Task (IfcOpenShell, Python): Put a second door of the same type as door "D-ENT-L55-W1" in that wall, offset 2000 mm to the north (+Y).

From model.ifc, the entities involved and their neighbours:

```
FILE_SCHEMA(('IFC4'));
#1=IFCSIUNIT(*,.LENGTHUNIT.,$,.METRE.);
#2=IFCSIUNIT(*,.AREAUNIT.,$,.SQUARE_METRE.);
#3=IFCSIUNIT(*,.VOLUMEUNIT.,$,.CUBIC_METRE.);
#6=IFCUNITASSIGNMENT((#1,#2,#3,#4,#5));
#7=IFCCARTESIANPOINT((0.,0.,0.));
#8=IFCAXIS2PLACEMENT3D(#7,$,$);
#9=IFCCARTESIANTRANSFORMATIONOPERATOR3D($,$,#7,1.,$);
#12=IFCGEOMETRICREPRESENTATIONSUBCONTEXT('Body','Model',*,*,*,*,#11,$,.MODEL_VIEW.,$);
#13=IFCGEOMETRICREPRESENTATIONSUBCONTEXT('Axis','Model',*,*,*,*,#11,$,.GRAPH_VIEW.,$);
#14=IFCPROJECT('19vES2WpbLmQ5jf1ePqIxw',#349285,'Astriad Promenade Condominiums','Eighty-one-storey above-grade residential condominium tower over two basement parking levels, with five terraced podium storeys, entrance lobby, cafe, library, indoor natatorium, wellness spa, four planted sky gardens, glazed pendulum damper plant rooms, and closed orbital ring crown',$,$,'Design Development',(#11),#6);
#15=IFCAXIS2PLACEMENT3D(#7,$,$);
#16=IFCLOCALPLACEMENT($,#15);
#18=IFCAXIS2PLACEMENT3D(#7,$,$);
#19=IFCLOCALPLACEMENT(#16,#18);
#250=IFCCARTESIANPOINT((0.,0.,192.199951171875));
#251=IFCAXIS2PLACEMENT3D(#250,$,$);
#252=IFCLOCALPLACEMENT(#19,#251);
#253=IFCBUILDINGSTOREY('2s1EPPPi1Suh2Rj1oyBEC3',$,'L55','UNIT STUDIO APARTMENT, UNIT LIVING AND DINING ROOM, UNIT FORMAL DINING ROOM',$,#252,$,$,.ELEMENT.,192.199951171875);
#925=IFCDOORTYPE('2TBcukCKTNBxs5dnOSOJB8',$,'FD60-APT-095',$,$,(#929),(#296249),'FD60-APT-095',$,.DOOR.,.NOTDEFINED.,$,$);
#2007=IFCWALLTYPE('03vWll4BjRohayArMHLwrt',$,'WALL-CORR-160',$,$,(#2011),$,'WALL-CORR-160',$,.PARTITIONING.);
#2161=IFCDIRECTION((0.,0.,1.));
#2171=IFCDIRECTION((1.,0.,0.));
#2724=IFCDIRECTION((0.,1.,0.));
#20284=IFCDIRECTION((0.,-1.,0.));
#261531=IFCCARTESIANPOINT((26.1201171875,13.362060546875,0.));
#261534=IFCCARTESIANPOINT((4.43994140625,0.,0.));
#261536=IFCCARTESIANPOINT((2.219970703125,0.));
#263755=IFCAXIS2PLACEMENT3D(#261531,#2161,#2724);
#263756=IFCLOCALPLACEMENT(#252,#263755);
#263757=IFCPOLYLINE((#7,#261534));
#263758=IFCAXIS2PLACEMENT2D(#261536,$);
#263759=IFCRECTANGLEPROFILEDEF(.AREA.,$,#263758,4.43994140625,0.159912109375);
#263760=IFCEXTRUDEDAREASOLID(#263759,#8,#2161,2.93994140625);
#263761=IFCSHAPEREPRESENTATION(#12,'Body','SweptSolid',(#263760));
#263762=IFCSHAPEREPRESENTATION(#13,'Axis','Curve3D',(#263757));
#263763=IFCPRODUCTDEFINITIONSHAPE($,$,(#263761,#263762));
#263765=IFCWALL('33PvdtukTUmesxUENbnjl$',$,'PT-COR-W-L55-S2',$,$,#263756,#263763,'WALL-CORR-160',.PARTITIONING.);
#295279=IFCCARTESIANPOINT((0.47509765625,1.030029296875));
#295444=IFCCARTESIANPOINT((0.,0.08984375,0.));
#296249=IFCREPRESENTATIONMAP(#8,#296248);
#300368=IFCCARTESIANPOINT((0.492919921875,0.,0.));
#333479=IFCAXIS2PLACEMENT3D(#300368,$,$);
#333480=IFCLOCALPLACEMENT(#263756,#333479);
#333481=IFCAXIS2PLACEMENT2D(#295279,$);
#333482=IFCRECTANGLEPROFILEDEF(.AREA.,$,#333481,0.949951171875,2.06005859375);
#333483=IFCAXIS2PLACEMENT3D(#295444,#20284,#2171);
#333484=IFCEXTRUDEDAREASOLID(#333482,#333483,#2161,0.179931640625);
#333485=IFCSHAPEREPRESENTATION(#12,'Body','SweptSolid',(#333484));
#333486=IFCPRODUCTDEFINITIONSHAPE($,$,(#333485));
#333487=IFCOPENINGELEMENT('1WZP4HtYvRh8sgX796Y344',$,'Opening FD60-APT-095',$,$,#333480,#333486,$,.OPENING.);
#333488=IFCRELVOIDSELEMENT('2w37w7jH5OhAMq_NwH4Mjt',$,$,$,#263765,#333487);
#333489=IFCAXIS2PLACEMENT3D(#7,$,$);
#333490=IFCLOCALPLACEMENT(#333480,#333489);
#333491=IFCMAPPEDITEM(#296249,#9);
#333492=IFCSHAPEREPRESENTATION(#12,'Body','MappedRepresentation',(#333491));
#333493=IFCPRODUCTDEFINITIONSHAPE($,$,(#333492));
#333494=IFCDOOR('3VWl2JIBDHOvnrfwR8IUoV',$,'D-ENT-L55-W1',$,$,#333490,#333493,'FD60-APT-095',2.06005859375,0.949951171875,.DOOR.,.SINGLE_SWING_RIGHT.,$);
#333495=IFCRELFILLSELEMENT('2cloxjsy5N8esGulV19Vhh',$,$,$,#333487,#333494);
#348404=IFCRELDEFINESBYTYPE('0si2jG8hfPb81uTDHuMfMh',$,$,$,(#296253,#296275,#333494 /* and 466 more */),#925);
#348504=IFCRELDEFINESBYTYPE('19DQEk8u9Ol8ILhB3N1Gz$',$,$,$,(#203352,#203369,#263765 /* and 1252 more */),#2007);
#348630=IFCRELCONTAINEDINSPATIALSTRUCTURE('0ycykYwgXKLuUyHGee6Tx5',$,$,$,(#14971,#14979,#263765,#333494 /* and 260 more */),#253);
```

```python
import ifcopenshell
import ifcopenshell.api.feature
import ifcopenshell.api.geometry
import ifcopenshell.api.root
import ifcopenshell.geom
import ifcopenshell.util.element
import ifcopenshell.util.placement
import ifcopenshell.util.shape
import ifcopenshell.util.unit

model = ifcopenshell.open("model.ifc")
unit_scale = ifcopenshell.util.unit.calculate_unit_scale(model)
settings = ifcopenshell.geom.settings()


def volume(element):
    """Net volume in cubic metres, openings subtracted."""
    shape = ifcopenshell.geom.create_shape(settings, element)
    return ifcopenshell.util.shape.get_volume(shape.geometry)


door = model.by_guid("3VWl2JIBDHOvnrfwR8IUoV")
opening = door.FillsVoids[0].RelatingOpeningElement
wall = opening.VoidsElements[0].RelatingBuildingElement
before = volume(wall)
shift = ifcopenshell.util.placement.get_local_placement(wall.ObjectPlacement)[:3, 0] * 2 / unit_scale

# copy_class copies the void relationship, type, container and properties, but no geometry.
new_opening = ifcopenshell.api.root.copy_class(model, product=opening)
new_opening.Representation = ifcopenshell.util.element.copy_deep(
    model, opening.Representation, exclude=["IfcGeometricRepresentationContext", "IfcRepresentationMap"]
)
new_door = ifcopenshell.api.root.copy_class(model, product=door)
new_door.Representation = ifcopenshell.util.element.copy_deep(
    model, door.Representation, exclude=["IfcGeometricRepresentationContext", "IfcRepresentationMap"]
)
new_door.Tag = None
ifcopenshell.api.feature.add_filling(model, opening=new_opening, element=new_door)

for old, new in ((opening, new_opening), (door, new_door)):
    matrix = ifcopenshell.util.placement.get_local_placement(old.ObjectPlacement)
    matrix[:3, 3] += shift
    ifcopenshell.api.geometry.edit_object_placement(model, product=new, matrix=matrix, is_si=False)

after = volume(wall)

print(f"wall volume {before:.3f} -> {after:.3f} m3")

model.write("model-out.ifc")
```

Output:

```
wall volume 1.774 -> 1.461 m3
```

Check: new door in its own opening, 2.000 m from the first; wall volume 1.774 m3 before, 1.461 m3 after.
